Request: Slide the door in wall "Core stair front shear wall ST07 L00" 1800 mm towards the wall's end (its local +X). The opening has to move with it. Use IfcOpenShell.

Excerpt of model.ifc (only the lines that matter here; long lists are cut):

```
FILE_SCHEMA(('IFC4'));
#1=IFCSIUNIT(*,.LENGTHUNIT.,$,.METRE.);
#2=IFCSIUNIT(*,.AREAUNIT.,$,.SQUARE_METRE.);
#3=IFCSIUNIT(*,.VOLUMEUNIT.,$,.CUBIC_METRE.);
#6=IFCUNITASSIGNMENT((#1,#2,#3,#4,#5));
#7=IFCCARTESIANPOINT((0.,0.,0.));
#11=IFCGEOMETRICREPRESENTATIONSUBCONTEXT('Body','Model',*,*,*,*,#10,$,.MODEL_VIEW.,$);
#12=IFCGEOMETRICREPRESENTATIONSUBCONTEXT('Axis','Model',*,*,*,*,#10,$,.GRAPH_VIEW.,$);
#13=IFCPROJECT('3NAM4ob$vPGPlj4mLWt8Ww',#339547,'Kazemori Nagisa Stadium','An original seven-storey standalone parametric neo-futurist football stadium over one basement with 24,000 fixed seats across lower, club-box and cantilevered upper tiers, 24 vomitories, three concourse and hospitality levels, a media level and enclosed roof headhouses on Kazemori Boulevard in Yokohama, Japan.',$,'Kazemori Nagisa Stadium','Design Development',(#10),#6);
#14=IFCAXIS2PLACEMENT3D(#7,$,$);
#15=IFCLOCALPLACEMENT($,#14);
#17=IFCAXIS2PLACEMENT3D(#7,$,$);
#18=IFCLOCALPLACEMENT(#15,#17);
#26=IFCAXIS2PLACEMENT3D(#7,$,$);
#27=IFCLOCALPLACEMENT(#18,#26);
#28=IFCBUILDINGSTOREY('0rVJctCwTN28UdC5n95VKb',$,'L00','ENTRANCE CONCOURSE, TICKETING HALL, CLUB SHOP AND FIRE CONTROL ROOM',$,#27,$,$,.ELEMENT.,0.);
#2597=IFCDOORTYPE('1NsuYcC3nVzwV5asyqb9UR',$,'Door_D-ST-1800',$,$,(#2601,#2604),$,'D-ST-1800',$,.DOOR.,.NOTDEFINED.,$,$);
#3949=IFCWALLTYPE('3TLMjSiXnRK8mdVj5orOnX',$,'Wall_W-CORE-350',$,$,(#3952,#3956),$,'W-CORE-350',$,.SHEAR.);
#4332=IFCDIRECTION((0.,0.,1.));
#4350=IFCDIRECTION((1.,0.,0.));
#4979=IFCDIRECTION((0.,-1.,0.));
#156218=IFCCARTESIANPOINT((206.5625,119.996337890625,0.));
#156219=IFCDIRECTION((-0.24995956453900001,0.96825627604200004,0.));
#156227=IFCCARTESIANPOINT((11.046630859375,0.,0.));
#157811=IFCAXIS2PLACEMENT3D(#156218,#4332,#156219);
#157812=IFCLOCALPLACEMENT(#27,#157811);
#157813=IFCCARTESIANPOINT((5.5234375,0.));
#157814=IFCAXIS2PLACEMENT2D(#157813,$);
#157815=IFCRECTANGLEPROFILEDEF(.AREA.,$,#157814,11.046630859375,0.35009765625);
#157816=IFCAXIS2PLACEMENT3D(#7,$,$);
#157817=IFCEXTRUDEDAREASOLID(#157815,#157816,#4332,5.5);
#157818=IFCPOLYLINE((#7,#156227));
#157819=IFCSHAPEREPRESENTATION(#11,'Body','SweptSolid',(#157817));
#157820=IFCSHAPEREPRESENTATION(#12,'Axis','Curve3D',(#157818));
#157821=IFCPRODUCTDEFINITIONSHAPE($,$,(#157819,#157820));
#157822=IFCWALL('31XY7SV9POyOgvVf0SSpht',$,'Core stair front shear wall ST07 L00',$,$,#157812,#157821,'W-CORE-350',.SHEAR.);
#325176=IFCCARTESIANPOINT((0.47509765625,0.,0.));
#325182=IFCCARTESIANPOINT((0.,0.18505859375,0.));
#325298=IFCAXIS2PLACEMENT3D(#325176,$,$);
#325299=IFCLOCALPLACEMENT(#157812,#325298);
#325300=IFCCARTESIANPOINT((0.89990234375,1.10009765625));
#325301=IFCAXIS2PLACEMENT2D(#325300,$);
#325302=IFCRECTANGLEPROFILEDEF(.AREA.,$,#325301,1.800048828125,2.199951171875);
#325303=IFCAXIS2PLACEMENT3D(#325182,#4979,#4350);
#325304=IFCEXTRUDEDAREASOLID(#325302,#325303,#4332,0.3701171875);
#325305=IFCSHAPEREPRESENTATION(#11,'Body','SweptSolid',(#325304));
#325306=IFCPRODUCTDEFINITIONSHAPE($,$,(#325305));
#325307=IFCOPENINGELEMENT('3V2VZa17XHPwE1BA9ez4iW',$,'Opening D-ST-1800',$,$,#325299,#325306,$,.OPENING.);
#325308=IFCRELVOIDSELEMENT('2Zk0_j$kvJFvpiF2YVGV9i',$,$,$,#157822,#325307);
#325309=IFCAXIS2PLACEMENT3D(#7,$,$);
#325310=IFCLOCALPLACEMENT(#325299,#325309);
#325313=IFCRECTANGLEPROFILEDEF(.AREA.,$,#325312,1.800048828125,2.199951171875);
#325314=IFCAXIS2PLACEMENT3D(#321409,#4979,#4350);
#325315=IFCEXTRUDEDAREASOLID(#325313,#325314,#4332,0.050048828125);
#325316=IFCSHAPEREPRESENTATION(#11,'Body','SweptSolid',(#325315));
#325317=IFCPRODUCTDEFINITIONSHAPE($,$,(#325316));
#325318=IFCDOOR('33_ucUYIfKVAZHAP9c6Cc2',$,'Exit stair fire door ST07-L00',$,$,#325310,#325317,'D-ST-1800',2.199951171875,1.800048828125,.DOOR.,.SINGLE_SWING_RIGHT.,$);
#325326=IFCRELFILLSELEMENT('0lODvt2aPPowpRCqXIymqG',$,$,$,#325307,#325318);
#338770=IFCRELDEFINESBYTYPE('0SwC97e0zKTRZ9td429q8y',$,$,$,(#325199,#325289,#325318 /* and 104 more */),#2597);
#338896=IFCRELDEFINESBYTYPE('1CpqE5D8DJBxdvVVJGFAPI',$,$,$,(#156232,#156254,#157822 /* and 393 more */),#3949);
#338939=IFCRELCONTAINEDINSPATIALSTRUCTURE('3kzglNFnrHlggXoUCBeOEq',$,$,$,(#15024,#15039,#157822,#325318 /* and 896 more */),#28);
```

```python
import ifcopenshell
import ifcopenshell.api.geometry
import ifcopenshell.util.placement

model = ifcopenshell.open("model.ifc")

door = model.by_id(325318)
opening = door.FillsVoids[0].RelatingOpeningElement
wall = opening.VoidsElements[0].RelatingBuildingElement

wall_matrix = ifcopenshell.util.placement.get_local_placement(wall.ObjectPlacement)
shift = wall_matrix[:3, 0] * 1.8
before = ifcopenshell.util.placement.get_local_placement(door.ObjectPlacement)[:3, 3].copy()

# The door is placed relative to its opening, so it follows when the opening moves.
matrix = ifcopenshell.util.placement.get_local_placement(opening.ObjectPlacement)
matrix[:3, 3] += shift
ifcopenshell.api.geometry.edit_object_placement(
    model, product=opening, matrix=matrix, is_si=False, should_transform_children=True
)

after = ifcopenshell.util.placement.get_local_placement(door.ObjectPlacement)[:3, 3]
print("door moved by", (after - before).round(3) + 0.0)

model.write("model_v2.ifc")
```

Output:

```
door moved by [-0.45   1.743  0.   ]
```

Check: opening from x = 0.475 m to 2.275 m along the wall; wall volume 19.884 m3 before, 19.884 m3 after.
